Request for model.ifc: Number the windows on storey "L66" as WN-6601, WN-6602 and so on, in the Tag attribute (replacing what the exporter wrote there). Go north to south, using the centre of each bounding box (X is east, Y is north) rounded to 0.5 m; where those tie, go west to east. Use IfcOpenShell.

First a look at what the model holds.

```python
import ifcopenshell
import ifcopenshell.util.element
import ifcopenshell.util.placement

model = ifcopenshell.open("model.ifc")
print(model.schema)
storey = next(s for s in model.by_type("IfcBuildingStorey") if s.Name == "L66")
windows = [e for e in ifcopenshell.util.element.get_decomposition(storey) if e.is_a("IfcWindow")]
for e in sorted(windows, key=lambda e: e.id()):
    origin = ifcopenshell.util.placement.get_local_placement(e.ObjectPlacement)[:3, 3]
    print(e.id(), e.Tag, e.Name, origin.round(2) + 0.0, sep=" | ")
```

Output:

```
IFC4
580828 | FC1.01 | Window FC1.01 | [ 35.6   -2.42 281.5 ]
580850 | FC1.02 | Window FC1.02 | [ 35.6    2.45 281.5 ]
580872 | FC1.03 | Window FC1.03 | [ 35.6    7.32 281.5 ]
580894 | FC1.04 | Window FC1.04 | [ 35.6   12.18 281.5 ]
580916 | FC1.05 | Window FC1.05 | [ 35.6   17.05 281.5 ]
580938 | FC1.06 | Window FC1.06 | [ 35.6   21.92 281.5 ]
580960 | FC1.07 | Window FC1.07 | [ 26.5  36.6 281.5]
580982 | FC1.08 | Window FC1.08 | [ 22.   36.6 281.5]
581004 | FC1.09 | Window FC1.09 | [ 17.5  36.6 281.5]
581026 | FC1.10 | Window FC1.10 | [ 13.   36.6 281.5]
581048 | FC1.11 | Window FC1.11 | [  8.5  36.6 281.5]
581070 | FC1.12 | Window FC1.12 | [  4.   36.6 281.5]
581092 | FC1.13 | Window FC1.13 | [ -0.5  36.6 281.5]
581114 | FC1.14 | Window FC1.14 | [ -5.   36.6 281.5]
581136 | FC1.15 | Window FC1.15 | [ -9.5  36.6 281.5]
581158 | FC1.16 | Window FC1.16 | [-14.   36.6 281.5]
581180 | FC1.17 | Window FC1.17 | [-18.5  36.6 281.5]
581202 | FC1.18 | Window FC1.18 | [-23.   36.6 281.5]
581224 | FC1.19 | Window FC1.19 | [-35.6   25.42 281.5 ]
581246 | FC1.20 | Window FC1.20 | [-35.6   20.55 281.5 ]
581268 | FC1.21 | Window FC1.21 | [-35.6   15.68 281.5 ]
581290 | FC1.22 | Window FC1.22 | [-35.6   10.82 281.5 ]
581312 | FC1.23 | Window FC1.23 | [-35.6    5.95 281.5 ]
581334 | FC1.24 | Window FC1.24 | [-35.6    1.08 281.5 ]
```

```python
import ifcopenshell
import ifcopenshell.geom
import ifcopenshell.util.element
import ifcopenshell.util.shape

model = ifcopenshell.open("model.ifc")
settings = ifcopenshell.geom.settings()
settings.set("use-world-coords", True)


def centre(element):
    shape = ifcopenshell.geom.create_shape(settings, element)
    return ifcopenshell.util.shape.get_bbox_centroid(shape.geometry)


storey = next(s for s in model.by_type("IfcBuildingStorey") if s.Name == "L66")
windows = [e for e in ifcopenshell.util.element.get_decomposition(storey) if e.is_a("IfcWindow")]

# Insertion points can sit at a corner or the storey origin, so sort by the geometry (in metres).
centres = {e: centre(e) for e in windows}
windows.sort(key=lambda e: (-round(centres[e][1] / 0.5), centres[e][0]))

for i, e in enumerate(windows, start=1):
    number = f"WN-66{i:02d}"
    e.Tag = number
    print(e.id(), number)

model.write("model_rev.ifc")
```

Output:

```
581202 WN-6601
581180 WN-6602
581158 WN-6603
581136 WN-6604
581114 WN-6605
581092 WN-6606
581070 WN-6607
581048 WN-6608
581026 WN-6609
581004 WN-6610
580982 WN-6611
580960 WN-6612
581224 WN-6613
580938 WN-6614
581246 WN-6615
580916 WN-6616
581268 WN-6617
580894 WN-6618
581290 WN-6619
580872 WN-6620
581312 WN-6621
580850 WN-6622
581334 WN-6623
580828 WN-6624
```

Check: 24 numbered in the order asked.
